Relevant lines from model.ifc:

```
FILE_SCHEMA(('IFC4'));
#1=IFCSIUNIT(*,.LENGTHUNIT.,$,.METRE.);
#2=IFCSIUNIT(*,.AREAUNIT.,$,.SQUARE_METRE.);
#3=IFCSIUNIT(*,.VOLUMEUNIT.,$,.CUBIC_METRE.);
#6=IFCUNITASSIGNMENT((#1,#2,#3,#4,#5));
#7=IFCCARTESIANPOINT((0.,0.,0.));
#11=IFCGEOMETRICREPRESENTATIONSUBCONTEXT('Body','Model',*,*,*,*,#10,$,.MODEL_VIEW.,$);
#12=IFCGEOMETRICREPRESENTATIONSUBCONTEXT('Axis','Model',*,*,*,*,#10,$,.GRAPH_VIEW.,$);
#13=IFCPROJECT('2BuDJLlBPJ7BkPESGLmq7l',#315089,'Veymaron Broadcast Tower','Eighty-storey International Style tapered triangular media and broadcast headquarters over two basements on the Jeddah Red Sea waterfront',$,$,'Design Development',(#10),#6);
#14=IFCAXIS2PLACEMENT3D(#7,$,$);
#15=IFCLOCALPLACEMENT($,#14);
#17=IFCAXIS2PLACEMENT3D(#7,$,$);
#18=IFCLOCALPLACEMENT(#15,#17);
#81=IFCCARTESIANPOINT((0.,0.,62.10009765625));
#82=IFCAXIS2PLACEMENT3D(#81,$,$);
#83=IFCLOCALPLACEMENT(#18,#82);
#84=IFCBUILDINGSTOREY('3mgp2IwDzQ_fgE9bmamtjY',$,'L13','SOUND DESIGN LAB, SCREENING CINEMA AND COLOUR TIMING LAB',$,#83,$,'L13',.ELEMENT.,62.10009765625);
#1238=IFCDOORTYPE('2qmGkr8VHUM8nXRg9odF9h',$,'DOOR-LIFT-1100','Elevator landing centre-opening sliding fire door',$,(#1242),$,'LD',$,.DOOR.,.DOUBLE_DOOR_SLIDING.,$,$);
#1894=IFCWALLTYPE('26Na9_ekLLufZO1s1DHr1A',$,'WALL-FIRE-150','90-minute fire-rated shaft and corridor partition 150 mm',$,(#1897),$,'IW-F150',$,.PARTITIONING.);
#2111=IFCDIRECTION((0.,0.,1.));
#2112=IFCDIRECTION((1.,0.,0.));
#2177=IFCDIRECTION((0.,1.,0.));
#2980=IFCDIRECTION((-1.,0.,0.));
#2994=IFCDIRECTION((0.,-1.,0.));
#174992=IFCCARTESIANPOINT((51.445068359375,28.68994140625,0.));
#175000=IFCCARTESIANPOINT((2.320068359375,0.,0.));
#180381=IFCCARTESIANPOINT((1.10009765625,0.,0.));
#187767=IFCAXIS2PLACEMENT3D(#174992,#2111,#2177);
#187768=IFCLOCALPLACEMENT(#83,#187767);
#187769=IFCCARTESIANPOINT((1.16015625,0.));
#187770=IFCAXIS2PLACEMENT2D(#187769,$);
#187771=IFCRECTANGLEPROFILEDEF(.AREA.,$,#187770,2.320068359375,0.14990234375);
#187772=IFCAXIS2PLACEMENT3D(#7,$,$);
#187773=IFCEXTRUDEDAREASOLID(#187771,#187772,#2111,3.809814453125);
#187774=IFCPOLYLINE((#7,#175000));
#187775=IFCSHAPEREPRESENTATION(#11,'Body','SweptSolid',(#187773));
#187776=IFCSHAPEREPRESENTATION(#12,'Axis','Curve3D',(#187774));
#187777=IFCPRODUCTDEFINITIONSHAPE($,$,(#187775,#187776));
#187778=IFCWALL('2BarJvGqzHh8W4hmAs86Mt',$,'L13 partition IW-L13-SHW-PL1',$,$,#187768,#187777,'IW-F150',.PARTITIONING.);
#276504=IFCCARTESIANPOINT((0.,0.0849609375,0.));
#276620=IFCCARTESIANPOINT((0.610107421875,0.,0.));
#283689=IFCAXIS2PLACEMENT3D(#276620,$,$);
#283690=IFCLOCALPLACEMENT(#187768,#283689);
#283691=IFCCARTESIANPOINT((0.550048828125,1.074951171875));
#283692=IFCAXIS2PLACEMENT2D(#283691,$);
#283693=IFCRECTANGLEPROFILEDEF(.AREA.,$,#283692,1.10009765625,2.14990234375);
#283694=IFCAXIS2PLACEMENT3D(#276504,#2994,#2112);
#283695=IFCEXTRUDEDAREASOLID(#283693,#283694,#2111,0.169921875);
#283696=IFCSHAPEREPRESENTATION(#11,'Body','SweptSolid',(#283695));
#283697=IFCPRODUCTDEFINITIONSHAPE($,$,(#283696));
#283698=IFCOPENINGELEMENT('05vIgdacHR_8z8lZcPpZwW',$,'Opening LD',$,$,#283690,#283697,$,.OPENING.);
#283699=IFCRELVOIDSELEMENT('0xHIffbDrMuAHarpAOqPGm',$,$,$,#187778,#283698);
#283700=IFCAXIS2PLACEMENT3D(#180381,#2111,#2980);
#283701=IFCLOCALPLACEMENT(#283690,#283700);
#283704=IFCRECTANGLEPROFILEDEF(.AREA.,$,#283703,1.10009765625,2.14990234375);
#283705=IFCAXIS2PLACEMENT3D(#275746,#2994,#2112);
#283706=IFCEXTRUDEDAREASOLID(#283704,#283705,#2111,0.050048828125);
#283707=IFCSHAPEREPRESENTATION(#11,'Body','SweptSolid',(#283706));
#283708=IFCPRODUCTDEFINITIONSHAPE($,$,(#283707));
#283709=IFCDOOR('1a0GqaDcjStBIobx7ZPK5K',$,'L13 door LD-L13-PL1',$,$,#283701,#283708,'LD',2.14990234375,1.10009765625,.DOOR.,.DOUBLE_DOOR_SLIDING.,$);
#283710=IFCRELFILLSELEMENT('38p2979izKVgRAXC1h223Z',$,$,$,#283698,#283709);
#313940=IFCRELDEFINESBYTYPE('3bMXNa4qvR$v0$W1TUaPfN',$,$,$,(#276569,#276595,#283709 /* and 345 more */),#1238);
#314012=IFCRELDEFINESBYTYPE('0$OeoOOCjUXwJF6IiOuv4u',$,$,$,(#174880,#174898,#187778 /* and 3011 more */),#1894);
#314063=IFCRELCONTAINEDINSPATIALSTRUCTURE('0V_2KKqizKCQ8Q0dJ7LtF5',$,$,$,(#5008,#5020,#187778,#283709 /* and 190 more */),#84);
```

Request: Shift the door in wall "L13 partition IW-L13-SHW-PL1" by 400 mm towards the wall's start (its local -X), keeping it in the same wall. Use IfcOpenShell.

```python
import ifcopenshell
import ifcopenshell.api.geometry
import ifcopenshell.util.placement
import ifcopenshell.util.unit

model = ifcopenshell.open("model.ifc")
unit_scale = ifcopenshell.util.unit.calculate_unit_scale(model)

door = model.by_guid("1a0GqaDcjStBIobx7ZPK5K")
opening = door.FillsVoids[0].RelatingOpeningElement
wall = opening.VoidsElements[0].RelatingBuildingElement

wall_matrix = ifcopenshell.util.placement.get_local_placement(wall.ObjectPlacement)
shift = wall_matrix[:3, 0] * -0.4 / unit_scale
before = ifcopenshell.util.placement.get_local_placement(door.ObjectPlacement)[:3, 3].copy()

# The door is placed relative to its opening, so it follows when the opening moves.
matrix = ifcopenshell.util.placement.get_local_placement(opening.ObjectPlacement)
matrix[:3, 3] += shift
ifcopenshell.api.geometry.edit_object_placement(
    model, product=opening, matrix=matrix, is_si=False, should_transform_children=True
)

after = ifcopenshell.util.placement.get_local_placement(door.ObjectPlacement)[:3, 3]
print("door moved by", (after - before).round(3) + 0.0)

model.write("model_rev.ifc")
```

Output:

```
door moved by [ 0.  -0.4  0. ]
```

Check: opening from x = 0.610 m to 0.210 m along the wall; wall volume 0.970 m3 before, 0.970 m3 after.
